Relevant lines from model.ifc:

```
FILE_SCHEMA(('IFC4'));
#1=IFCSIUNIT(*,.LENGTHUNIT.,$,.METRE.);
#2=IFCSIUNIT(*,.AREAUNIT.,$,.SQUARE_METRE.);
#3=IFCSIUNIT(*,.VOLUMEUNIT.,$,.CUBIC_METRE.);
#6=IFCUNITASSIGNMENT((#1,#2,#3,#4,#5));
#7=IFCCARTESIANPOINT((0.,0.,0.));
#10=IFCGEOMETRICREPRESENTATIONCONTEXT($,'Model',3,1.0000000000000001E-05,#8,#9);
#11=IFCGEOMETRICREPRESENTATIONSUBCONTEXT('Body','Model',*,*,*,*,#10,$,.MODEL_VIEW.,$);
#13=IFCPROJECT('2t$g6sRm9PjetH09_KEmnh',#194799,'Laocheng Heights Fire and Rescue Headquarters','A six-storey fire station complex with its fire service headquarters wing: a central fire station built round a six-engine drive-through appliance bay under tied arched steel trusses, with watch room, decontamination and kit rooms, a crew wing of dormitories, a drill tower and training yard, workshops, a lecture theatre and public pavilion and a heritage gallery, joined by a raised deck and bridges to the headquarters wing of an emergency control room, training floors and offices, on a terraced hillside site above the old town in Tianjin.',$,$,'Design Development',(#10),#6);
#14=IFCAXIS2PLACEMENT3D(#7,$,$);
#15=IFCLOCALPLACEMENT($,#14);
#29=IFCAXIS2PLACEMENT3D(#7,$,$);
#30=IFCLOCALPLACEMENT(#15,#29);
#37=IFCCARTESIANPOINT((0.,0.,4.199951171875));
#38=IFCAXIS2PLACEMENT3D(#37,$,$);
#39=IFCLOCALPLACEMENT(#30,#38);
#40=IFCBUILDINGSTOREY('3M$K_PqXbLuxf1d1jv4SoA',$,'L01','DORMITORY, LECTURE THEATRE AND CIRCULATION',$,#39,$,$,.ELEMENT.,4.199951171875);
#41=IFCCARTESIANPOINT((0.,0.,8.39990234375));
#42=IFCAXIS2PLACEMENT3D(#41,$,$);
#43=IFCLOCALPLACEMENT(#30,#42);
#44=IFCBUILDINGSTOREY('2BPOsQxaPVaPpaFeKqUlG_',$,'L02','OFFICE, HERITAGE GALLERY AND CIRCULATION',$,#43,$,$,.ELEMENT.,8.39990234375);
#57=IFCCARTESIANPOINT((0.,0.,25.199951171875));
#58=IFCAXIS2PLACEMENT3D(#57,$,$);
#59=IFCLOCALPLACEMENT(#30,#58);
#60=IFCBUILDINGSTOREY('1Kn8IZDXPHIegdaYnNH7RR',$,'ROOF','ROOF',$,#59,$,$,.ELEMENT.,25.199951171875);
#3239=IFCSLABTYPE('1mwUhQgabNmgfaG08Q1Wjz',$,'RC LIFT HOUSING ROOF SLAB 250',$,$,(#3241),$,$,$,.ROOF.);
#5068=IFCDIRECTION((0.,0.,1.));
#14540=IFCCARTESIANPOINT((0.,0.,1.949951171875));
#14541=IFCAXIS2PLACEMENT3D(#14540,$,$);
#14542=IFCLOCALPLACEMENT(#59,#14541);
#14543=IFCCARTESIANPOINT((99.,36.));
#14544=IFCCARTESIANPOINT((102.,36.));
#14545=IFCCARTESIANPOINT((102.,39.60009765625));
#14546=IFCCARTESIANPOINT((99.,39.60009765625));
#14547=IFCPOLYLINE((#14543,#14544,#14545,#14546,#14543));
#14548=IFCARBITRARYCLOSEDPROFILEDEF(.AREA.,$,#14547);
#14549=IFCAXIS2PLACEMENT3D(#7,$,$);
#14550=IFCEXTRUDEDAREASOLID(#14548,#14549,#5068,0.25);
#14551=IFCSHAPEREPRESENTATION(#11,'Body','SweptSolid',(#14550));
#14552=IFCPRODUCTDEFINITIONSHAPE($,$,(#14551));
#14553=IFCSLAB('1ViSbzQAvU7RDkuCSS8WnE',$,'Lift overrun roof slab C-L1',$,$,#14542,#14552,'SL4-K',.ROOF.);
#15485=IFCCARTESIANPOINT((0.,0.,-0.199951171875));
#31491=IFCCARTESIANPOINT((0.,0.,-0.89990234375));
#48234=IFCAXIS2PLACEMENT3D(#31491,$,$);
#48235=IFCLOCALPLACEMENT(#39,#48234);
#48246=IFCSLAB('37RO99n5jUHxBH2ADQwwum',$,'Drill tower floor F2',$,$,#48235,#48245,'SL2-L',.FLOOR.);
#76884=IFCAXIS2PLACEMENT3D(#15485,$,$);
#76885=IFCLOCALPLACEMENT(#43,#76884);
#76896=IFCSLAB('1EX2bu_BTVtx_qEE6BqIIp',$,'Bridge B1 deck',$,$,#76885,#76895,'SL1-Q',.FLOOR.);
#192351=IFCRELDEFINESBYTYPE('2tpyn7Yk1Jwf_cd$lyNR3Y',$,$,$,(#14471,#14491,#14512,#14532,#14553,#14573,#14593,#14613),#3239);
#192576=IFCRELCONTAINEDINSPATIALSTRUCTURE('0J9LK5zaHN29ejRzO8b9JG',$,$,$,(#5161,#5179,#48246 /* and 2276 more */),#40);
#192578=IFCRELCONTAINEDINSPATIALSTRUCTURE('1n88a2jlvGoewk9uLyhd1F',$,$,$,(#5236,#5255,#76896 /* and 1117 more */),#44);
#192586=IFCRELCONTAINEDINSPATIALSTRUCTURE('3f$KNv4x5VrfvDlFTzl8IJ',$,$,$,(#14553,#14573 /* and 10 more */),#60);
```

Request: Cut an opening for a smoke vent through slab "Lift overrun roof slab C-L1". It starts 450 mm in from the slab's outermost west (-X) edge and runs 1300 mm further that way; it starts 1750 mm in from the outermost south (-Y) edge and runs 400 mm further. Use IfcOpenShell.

```python
import numpy as np
import ifcopenshell
import ifcopenshell.api.feature
import ifcopenshell.api.geometry
import ifcopenshell.api.root
import ifcopenshell.geom
import ifcopenshell.util.placement
import ifcopenshell.util.representation
import ifcopenshell.util.shape
import ifcopenshell.util.unit

model = ifcopenshell.open("model.ifc")
unit_scale = ifcopenshell.util.unit.calculate_unit_scale(model)
settings = ifcopenshell.geom.settings()


def volume(element):
    """Net volume in cubic metres, openings subtracted."""
    shape = ifcopenshell.geom.create_shape(settings, element)
    return ifcopenshell.util.shape.get_volume(shape.geometry)


slab = model.by_guid("1ViSbzQAvU7RDkuCSS8WnE")
before = volume(slab)

# Extent in the slab's own axes, in metres. The edges named are its -X and -Y sides.
slab_shape = ifcopenshell.geom.create_shape(settings, slab)
vertices = ifcopenshell.util.shape.get_vertices(slab_shape.geometry)
x_min, y_min, bottom = vertices.min(axis=0)
top = vertices[:, 2].max()

opening = ifcopenshell.api.root.create_entity(model, ifc_class="IfcOpeningElement", name="Smoke vent opening", predefined_type="OPENING")
context = ifcopenshell.util.representation.get_context(model, "Model", "Body", "MODEL_VIEW")
width, depth = 1.3, 0.4
outline = [(0.0, 0.0), (width, 0.0), (width, depth), (0.0, depth), (0.0, 0.0)]
# Overshoot both faces by 50 mm so the cut is clean.
shape = ifcopenshell.api.geometry.add_slab_representation(
    model, context=context, depth=top - bottom + 0.1, polyline=outline
)
ifcopenshell.api.geometry.assign_representation(model, product=opening, representation=shape)

matrix = ifcopenshell.util.placement.get_local_placement(slab.ObjectPlacement)
matrix[:, 3] = matrix @ np.append(np.array([x_min + 0.45, y_min + 1.75, bottom - 0.05]) / unit_scale, 1.0)
ifcopenshell.api.geometry.edit_object_placement(model, product=opening, matrix=matrix, is_si=False)
ifcopenshell.api.feature.add_feature(model, feature=opening, element=slab)

after = volume(slab)

print(f"slab volume {before:.3f} -> {after:.3f} m3")

model.write("model_rev.ifc")
```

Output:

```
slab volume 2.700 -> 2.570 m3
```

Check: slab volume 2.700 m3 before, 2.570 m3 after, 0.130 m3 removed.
